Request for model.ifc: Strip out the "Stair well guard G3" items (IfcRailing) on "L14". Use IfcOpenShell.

First a look at what the model holds.

```python
import ifcopenshell
import ifcopenshell.util.element

model = ifcopenshell.open("model.ifc")
print(model.schema)
storey = next(s for s in model.by_type("IfcBuildingStorey") if s.Name == "L14")
railings = [e for e in ifcopenshell.util.element.get_decomposition(storey) if e.is_a("IfcRailing")]
seen = {}
for e in railings:
    element_type = ifcopenshell.util.element.get_type(e)
    name = element_type.Name if element_type not in (None, e) else None
    seen[name] = seen.get(name, 0) + 1
for name, count in sorted(seen.items(), key=str):
    print(count, "x", name)
```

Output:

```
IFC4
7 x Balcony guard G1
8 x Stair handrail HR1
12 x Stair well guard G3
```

```python
import ifcopenshell
import ifcopenshell.api.root
import ifcopenshell.util.element

model = ifcopenshell.open("model.ifc")

storey = next(s for s in model.by_type("IfcBuildingStorey") if s.Name == "L14")
railings = [e for e in ifcopenshell.util.element.get_decomposition(storey) if e.is_a("IfcRailing")]
targets = [e for e in railings if (t := ifcopenshell.util.element.get_type(e)) not in (None, e) and t.Name == "Stair well guard G3"]

for e in targets:
    ifcopenshell.api.root.remove_product(model, product=e)
print(len(targets), "removed")

model.write("model_rev.ifc")
```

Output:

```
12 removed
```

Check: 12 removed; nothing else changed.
